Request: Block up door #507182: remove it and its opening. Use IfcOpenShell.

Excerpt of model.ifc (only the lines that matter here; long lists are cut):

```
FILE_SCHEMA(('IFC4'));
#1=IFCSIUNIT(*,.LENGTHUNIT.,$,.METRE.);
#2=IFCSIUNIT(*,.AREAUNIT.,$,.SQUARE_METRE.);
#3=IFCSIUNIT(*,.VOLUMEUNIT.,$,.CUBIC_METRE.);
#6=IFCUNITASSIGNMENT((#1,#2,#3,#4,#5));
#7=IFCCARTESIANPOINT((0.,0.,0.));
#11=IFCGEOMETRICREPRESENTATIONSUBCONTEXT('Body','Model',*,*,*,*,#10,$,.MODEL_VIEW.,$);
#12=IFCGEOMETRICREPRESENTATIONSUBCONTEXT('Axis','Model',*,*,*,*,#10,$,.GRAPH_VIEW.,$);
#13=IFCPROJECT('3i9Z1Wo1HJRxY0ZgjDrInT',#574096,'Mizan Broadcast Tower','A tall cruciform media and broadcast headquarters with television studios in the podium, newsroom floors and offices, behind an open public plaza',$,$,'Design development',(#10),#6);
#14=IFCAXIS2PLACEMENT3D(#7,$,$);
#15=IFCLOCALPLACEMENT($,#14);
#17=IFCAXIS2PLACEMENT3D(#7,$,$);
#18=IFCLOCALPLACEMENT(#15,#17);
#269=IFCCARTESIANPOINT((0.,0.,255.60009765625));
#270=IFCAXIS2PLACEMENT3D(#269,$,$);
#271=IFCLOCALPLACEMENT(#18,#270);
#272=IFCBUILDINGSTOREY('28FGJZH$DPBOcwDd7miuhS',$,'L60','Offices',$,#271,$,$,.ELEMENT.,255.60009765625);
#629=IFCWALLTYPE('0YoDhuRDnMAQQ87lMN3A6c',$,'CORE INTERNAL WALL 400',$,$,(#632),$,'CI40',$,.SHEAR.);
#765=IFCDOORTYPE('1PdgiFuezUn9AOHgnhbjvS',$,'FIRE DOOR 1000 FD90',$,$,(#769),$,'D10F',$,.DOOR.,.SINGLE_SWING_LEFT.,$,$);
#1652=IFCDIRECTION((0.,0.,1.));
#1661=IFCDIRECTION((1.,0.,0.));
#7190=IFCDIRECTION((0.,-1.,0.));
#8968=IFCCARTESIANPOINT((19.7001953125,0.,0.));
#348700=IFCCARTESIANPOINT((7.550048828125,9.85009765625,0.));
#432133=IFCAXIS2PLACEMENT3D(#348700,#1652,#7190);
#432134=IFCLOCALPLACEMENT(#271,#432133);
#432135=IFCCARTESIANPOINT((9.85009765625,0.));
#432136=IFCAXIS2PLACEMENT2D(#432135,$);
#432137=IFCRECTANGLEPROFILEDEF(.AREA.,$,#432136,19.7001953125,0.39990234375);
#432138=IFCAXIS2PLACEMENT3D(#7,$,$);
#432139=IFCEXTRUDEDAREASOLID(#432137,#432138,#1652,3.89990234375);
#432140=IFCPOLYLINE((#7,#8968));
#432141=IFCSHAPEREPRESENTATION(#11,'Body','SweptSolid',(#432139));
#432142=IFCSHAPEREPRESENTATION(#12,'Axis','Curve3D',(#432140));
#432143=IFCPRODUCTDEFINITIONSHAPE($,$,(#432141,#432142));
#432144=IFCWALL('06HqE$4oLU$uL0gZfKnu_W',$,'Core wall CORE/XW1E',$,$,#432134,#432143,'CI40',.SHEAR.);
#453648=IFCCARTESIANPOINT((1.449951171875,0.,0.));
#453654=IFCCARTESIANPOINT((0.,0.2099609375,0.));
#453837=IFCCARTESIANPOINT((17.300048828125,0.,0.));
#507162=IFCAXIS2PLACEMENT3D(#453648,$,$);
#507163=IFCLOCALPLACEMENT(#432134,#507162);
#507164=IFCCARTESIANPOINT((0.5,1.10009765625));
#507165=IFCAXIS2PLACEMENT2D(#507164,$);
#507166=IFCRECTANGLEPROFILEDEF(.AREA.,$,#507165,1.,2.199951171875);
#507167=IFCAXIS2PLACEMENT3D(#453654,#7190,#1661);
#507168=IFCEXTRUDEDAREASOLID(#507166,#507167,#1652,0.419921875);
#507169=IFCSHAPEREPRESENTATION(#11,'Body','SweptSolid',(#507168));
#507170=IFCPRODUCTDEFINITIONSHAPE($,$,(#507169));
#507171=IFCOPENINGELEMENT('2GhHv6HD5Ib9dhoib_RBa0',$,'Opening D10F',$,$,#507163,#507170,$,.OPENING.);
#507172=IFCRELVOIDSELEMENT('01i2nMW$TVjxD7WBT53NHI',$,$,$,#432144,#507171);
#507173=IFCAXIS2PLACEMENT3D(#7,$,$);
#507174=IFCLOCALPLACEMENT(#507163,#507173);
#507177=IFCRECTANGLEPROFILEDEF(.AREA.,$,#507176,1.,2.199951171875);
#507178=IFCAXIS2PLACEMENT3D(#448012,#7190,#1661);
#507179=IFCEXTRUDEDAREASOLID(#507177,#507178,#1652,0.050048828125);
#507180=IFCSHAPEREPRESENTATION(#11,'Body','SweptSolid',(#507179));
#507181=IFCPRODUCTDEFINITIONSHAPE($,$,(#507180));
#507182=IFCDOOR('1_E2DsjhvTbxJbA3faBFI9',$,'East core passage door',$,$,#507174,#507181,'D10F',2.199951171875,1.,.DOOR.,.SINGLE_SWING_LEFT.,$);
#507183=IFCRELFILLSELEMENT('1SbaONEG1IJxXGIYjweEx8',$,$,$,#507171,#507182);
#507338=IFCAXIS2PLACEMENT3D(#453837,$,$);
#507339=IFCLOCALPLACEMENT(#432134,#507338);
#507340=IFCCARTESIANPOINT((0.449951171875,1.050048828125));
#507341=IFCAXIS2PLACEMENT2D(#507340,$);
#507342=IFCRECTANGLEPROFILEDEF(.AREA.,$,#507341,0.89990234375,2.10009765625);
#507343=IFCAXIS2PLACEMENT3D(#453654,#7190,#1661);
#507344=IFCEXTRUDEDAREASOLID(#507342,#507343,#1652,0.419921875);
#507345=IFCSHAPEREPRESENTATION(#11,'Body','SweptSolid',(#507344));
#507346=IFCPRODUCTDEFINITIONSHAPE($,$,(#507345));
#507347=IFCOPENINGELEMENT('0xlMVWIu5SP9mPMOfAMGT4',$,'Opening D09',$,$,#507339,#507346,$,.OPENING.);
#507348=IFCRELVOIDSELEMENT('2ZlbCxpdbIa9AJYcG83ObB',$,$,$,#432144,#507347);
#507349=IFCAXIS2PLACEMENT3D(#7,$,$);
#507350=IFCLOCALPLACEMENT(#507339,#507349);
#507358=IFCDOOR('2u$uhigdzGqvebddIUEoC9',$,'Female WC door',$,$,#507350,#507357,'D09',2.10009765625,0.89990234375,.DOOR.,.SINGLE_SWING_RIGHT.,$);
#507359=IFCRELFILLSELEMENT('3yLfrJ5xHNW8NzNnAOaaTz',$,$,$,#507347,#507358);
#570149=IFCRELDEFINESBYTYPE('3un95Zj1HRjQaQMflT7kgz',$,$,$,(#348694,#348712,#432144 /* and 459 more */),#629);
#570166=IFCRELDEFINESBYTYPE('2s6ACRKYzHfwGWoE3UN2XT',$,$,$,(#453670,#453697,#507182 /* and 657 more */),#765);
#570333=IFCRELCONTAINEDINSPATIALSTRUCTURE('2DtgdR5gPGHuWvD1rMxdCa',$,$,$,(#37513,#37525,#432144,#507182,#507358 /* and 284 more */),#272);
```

```python
import ifcopenshell
import ifcopenshell.api.feature
import ifcopenshell.api.root
import ifcopenshell.geom
import ifcopenshell.util.shape

model = ifcopenshell.open("model.ifc")
settings = ifcopenshell.geom.settings()


def volume(element):
    """Net volume in cubic metres, openings subtracted."""
    shape = ifcopenshell.geom.create_shape(settings, element)
    return ifcopenshell.util.shape.get_volume(shape.geometry)


door = model.by_id(507182)
opening = door.FillsVoids[0].RelatingOpeningElement
wall = opening.VoidsElements[0].RelatingBuildingElement
before = volume(wall)

ifcopenshell.api.root.remove_product(model, product=door)
ifcopenshell.api.feature.remove_feature(model, feature=opening)

after = volume(wall)

print(f"wall volume {before:.3f} -> {after:.3f} m3")

model.write("model_v2.ifc")
```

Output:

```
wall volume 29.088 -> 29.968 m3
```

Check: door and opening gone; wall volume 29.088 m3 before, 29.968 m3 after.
